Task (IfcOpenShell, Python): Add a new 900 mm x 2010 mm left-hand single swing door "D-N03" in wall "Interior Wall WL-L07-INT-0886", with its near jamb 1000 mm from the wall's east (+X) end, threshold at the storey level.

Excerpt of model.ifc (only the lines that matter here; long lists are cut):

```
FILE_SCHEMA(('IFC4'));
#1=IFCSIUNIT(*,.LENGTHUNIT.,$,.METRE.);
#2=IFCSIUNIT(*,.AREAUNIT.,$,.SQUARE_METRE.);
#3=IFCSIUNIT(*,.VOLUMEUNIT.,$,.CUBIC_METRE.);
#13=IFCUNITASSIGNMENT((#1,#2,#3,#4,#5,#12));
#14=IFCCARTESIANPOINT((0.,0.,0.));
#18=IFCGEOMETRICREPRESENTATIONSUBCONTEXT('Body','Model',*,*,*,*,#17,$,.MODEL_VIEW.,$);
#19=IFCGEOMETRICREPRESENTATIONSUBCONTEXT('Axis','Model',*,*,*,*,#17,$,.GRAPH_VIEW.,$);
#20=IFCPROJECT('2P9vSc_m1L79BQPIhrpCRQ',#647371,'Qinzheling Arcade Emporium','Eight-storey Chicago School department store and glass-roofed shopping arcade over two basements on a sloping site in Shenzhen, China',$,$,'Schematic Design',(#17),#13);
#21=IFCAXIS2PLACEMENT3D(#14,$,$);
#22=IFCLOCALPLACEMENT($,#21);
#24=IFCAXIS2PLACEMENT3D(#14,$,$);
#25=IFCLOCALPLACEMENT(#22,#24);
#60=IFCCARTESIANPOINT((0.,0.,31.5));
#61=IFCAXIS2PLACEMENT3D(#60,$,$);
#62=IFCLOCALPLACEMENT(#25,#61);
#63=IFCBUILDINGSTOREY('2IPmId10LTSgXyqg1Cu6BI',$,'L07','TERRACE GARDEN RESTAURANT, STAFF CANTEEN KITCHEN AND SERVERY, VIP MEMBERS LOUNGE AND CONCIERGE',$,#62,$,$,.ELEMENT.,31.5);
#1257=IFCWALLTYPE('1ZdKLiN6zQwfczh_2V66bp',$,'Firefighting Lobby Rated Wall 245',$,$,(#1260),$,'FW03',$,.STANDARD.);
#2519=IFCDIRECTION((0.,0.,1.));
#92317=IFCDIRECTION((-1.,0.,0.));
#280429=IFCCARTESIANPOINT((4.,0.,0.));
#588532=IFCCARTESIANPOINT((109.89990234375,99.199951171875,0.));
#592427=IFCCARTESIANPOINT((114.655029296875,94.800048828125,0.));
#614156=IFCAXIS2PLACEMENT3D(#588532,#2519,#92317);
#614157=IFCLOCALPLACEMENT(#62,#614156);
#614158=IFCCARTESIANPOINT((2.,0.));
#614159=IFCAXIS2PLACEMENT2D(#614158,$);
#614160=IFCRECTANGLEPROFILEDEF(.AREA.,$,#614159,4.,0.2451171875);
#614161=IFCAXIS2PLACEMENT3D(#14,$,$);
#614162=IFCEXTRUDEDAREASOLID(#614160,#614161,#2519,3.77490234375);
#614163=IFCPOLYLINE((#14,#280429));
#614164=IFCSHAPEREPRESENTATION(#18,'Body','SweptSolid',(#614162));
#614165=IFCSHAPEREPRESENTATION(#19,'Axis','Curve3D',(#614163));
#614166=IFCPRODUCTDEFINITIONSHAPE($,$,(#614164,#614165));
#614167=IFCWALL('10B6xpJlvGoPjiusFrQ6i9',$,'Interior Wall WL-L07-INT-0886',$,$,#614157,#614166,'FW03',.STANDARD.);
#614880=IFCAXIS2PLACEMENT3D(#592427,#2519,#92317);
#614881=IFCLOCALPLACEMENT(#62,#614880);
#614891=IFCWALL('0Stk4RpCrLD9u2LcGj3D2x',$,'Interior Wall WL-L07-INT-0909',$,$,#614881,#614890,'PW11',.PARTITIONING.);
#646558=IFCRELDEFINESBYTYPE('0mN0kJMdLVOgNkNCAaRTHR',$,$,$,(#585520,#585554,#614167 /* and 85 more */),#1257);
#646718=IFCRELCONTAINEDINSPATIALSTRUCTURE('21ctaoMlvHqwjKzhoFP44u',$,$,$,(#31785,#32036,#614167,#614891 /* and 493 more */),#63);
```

```python
import numpy as np
import ifcopenshell
import ifcopenshell.api.feature
import ifcopenshell.api.geometry
import ifcopenshell.api.root
import ifcopenshell.api.spatial
import ifcopenshell.geom
import ifcopenshell.util.element
import ifcopenshell.util.placement
import ifcopenshell.util.representation
import ifcopenshell.util.shape
import ifcopenshell.util.unit

model = ifcopenshell.open("model.ifc")
unit_scale = ifcopenshell.util.unit.calculate_unit_scale(model)
settings = ifcopenshell.geom.settings()


def volume(element):
    """Net volume in cubic metres, openings subtracted."""
    shape = ifcopenshell.geom.create_shape(settings, element)
    return ifcopenshell.util.shape.get_volume(shape.geometry)


wall = model.by_guid("10B6xpJlvGoPjiusFrQ6i9")
storey = ifcopenshell.util.element.get_container(wall, ifc_class="IfcBuildingStorey")
context = ifcopenshell.util.representation.get_context(model, "Model", "Body", "MODEL_VIEW")
before = volume(wall)

width, height, from_end, sill = 0.9, 2.01, 1, 0.0  # metres

# The wall runs along its own X axis, and the end named is its -X end.
wall_shape = ifcopenshell.geom.create_shape(settings, wall)
x, y, z = ifcopenshell.util.shape.get_vertices(wall_shape.geometry).T
start = x.min() + from_end
face, thickness = float(y.min()), float(y.max() - y.min())
wall_matrix = ifcopenshell.util.placement.get_local_placement(wall.ObjectPlacement)
level = ifcopenshell.util.placement.get_local_placement(storey.ObjectPlacement)[2, 3]


def in_wall(x, y):
    """Placement at x, y metres in the wall's axes, at sill height."""
    matrix = wall_matrix.copy()
    matrix[:, 3] = wall_matrix @ np.array([x / unit_scale, y / unit_scale, 0.0, 1.0])
    matrix[2, 3] = level + sill / unit_scale
    return matrix


# Opening: a box that overshoots both wall faces by 50 mm.
opening = ifcopenshell.api.root.create_entity(model, ifc_class="IfcOpeningElement", predefined_type="OPENING")
box = ifcopenshell.api.geometry.add_wall_representation(
    model, context=context, length=width, height=height, thickness=thickness + 0.1
)
ifcopenshell.api.geometry.assign_representation(model, product=opening, representation=box)
ifcopenshell.api.geometry.edit_object_placement(model, product=opening, matrix=in_wall(start, face - 0.05), is_si=False)
ifcopenshell.api.feature.add_feature(model, feature=opening, element=wall)

door = ifcopenshell.api.root.create_entity(model, ifc_class="IfcDoor", name="D-N03", predefined_type="DOOR")
door.OverallWidth, door.OverallHeight = width / unit_scale, height / unit_scale
door.OperationType = "SINGLE_SWING_LEFT"
body = ifcopenshell.api.geometry.add_door_representation(
    model,
    context=context,
    overall_width=door.OverallWidth,
    overall_height=door.OverallHeight,
    operation_type="SINGLE_SWING_LEFT",
    lining_properties={"LiningDepth": thickness / unit_scale, "ThresholdDepth": thickness / unit_scale},
)
ifcopenshell.api.geometry.assign_representation(model, product=door, representation=body)
ifcopenshell.api.spatial.assign_container(model, products=[door], relating_structure=storey)
ifcopenshell.api.feature.add_filling(model, opening=opening, element=door)

# The lining spans the wall, so the door starts at the wall face.
ifcopenshell.api.geometry.edit_object_placement(model, product=door, matrix=in_wall(start, face), is_si=False)

after = volume(wall)

print(f"wall volume {before:.3f} -> {after:.3f} m3")

model.write("model_v2.ifc")
```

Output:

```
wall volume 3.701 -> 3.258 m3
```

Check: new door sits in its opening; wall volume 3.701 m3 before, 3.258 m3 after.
